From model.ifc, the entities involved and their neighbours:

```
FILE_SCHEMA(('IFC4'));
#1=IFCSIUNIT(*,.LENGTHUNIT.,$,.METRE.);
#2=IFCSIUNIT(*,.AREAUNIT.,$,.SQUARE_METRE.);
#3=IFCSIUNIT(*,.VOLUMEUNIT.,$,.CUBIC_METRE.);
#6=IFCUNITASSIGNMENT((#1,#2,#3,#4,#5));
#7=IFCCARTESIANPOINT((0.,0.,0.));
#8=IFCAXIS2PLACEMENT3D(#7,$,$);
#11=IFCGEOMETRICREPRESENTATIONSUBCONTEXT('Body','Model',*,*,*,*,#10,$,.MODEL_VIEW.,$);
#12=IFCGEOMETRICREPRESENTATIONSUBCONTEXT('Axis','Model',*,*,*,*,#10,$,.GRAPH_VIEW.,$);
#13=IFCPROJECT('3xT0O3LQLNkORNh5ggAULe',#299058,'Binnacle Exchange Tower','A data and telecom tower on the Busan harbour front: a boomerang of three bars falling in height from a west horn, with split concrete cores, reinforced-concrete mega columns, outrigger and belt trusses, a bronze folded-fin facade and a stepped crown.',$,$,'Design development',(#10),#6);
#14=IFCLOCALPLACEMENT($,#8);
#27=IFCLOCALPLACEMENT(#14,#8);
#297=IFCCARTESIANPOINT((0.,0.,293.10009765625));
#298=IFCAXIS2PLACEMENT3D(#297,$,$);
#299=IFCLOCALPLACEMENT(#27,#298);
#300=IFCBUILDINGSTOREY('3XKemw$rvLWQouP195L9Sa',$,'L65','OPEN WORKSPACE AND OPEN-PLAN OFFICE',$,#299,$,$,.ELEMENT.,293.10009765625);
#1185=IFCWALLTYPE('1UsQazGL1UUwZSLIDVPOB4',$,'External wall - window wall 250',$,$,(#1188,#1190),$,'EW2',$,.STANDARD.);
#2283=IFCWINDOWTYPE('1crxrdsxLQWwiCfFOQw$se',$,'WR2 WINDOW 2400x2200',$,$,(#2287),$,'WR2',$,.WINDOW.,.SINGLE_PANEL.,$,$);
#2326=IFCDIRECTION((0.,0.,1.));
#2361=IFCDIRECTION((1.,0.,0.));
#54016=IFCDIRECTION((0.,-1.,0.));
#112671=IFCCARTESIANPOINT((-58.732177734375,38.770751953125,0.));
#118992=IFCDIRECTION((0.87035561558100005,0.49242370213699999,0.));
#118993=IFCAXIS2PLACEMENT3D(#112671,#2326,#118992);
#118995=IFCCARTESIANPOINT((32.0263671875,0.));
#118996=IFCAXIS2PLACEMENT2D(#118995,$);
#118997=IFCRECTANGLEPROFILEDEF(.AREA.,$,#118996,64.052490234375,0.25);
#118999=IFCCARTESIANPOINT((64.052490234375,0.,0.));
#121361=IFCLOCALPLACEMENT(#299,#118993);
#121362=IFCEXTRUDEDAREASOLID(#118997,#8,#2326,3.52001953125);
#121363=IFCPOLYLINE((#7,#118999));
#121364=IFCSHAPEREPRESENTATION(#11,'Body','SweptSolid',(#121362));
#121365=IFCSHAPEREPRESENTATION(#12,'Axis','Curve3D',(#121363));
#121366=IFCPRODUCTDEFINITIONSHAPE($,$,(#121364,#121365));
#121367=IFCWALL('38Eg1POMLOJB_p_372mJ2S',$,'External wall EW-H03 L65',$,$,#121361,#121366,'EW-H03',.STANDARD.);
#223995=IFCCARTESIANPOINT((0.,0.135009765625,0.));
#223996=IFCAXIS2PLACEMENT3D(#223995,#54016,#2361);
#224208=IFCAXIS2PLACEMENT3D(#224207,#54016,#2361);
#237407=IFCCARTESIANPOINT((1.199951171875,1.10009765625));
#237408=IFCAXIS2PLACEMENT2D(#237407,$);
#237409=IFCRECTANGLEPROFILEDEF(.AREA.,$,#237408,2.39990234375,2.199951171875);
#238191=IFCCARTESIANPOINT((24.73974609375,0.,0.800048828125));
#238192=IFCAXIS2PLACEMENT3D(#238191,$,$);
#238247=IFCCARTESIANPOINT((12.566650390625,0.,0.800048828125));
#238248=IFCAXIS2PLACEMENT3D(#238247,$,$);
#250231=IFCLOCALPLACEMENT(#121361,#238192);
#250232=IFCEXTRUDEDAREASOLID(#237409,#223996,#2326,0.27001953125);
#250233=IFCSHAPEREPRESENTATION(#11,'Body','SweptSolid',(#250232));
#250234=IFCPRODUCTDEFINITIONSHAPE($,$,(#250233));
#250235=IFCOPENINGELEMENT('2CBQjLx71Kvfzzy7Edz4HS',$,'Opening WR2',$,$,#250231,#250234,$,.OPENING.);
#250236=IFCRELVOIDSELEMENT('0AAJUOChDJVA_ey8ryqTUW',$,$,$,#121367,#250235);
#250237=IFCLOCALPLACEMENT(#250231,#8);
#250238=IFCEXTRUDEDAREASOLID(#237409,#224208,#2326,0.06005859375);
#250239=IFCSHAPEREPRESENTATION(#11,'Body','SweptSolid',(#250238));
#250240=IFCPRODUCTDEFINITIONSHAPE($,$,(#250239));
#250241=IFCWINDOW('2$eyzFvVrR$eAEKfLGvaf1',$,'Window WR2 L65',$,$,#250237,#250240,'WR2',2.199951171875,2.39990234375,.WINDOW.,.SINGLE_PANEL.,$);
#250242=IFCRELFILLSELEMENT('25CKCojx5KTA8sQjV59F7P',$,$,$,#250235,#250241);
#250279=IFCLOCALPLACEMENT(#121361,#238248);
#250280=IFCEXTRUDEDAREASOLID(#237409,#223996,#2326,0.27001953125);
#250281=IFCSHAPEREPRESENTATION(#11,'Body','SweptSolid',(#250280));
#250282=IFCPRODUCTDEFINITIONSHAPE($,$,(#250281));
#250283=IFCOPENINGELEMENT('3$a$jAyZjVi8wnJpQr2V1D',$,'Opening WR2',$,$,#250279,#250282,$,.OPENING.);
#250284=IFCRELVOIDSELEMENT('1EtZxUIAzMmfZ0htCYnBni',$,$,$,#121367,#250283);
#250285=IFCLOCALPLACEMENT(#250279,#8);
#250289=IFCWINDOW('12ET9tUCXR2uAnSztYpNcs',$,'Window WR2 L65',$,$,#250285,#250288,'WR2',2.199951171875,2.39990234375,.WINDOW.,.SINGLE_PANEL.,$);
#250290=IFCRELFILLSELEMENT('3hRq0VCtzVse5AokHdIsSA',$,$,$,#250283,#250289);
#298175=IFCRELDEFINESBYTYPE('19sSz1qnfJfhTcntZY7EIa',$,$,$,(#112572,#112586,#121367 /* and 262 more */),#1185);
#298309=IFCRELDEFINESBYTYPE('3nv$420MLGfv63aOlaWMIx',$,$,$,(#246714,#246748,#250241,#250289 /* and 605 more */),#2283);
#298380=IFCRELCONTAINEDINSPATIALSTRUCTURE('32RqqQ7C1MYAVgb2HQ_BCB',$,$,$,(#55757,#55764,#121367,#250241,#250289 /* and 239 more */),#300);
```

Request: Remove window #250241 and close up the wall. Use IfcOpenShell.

```python
import ifcopenshell
import ifcopenshell.api.feature
import ifcopenshell.api.root
import ifcopenshell.geom
import ifcopenshell.util.shape

model = ifcopenshell.open("model.ifc")
settings = ifcopenshell.geom.settings()


def volume(element):
    """Net volume in cubic metres, openings subtracted."""
    shape = ifcopenshell.geom.create_shape(settings, element)
    return ifcopenshell.util.shape.get_volume(shape.geometry)


window = model.by_id(250241)
opening = window.FillsVoids[0].RelatingOpeningElement
wall = opening.VoidsElements[0].RelatingBuildingElement
before = volume(wall)

ifcopenshell.api.root.remove_product(model, product=window)
ifcopenshell.api.feature.remove_feature(model, feature=opening)

after = volume(wall)

print(f"wall volume {before:.3f} -> {after:.3f} m3")

model.write("model-out.ifc")
```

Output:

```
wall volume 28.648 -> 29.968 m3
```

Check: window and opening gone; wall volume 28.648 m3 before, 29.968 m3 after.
